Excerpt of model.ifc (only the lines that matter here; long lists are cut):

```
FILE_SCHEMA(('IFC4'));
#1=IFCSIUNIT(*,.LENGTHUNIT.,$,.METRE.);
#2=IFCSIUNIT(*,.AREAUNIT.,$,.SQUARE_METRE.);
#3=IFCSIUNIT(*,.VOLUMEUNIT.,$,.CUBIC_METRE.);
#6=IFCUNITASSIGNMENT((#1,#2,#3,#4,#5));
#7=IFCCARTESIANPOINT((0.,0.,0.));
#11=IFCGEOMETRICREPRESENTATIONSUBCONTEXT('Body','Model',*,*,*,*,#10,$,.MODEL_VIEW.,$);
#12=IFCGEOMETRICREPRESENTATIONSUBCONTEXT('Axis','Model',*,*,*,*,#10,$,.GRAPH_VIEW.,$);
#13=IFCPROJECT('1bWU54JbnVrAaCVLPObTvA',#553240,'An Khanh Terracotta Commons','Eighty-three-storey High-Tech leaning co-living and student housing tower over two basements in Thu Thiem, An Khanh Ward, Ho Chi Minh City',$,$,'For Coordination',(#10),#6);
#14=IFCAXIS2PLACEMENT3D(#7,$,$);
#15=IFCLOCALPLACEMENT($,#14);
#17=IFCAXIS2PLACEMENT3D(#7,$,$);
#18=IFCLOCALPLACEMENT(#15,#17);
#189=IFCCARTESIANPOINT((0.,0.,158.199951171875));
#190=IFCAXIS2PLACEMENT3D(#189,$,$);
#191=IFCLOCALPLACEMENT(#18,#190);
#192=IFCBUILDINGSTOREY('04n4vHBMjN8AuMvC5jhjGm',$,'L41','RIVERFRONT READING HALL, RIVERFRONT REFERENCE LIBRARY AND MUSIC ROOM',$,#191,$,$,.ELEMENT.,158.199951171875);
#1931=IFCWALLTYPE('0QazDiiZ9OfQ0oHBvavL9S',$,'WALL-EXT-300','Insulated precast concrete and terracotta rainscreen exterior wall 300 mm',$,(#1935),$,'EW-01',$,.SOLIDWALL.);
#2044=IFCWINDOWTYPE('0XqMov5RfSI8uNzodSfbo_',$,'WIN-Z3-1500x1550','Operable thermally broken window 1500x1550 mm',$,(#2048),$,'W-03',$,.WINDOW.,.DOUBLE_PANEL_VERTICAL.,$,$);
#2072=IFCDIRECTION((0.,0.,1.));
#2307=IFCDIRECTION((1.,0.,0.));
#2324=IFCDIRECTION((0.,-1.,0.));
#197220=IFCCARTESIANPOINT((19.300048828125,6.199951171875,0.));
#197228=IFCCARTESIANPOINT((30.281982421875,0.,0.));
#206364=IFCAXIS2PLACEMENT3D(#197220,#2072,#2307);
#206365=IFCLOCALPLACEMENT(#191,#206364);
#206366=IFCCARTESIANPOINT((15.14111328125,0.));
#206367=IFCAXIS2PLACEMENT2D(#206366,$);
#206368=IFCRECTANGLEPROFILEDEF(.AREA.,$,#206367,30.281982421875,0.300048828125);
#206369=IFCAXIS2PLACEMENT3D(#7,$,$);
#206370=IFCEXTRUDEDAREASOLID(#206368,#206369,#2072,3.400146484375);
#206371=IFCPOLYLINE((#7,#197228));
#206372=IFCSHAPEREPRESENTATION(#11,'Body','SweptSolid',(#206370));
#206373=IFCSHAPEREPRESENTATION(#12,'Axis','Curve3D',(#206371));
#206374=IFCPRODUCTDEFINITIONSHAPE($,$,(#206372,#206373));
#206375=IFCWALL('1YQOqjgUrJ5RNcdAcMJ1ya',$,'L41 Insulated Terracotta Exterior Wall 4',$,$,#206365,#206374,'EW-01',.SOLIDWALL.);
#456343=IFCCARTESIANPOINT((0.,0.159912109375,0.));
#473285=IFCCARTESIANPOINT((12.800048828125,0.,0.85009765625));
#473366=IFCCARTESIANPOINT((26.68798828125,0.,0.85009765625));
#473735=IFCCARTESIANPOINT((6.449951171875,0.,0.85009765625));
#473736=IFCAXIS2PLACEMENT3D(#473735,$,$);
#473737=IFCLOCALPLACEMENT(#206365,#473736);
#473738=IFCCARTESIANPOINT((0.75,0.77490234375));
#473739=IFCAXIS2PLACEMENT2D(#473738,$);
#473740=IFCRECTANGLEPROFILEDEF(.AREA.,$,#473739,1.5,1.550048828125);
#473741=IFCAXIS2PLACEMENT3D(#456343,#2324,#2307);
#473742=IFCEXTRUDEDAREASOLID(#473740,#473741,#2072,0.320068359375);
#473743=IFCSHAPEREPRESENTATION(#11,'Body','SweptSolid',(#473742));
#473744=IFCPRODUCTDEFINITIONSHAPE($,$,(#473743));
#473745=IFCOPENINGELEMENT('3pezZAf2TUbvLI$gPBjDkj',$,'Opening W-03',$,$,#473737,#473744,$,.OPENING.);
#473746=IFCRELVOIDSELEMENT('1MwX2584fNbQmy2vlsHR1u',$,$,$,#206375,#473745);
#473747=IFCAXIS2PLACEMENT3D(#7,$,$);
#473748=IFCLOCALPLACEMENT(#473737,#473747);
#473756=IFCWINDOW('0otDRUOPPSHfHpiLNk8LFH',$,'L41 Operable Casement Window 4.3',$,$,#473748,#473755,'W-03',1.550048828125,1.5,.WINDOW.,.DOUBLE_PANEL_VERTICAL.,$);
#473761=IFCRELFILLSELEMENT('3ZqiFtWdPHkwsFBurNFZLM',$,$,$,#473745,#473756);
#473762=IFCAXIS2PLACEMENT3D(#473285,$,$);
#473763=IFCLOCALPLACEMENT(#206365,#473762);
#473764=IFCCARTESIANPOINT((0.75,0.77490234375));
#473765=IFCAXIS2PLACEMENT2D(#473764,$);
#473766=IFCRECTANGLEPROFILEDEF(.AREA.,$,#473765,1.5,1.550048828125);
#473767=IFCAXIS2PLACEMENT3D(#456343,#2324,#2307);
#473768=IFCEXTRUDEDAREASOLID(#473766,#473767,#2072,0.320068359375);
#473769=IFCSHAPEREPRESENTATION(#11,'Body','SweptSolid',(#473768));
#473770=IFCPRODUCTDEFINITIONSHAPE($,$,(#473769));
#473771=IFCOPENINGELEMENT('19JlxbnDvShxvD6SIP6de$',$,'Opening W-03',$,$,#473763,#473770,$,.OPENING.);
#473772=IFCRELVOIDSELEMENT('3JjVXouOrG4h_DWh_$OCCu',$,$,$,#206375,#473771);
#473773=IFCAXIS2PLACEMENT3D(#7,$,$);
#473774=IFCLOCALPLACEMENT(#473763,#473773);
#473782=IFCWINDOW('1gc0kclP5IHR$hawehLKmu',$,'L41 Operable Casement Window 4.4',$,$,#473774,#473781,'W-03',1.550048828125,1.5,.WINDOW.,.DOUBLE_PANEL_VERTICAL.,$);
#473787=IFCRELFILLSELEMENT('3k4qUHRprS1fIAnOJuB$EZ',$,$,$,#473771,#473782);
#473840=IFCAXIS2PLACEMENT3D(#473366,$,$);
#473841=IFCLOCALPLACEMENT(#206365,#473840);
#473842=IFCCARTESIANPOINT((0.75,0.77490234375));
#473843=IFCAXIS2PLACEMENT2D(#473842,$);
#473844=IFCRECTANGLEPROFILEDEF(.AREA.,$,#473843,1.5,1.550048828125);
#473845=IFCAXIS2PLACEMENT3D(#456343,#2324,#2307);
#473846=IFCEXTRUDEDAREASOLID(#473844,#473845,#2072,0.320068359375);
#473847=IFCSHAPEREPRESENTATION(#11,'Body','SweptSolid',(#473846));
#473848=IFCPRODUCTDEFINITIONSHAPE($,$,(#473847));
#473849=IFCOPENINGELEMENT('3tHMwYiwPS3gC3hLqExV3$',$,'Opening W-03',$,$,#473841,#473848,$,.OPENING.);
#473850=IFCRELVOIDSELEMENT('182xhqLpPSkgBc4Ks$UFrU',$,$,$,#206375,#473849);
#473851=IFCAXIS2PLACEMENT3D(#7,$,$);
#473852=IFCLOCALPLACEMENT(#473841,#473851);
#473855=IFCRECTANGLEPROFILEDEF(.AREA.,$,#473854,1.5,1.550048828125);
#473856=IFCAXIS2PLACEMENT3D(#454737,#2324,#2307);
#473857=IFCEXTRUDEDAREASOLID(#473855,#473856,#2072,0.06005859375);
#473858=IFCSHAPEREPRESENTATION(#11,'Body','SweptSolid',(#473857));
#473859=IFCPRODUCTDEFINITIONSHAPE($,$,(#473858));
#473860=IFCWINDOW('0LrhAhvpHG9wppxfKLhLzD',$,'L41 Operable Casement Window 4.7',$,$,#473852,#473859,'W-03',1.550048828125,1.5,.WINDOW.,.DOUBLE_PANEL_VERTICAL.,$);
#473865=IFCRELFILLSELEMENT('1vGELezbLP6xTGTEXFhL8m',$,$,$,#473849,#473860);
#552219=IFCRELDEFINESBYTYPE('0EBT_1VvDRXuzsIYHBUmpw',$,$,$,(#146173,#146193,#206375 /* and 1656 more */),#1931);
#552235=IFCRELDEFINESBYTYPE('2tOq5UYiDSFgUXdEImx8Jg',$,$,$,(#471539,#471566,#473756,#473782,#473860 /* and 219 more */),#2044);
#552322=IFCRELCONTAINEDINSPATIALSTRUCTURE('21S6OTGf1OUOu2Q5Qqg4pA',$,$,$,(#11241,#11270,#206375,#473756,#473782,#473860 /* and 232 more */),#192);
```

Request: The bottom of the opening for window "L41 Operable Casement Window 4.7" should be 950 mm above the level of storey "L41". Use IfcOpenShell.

```python
import numpy as np
import ifcopenshell
import ifcopenshell.api.geometry
import ifcopenshell.geom
import ifcopenshell.util.element
import ifcopenshell.util.placement
import ifcopenshell.util.shape
import ifcopenshell.util.unit

model = ifcopenshell.open("model.ifc")
unit_scale = ifcopenshell.util.unit.calculate_unit_scale(model)

window = model.by_guid("0LrhAhvpHG9wppxfKLhLzD")
opening = window.FillsVoids[0].RelatingOpeningElement
storey = ifcopenshell.util.element.get_container(window, ifc_class="IfcBuildingStorey")
level = ifcopenshell.util.placement.get_local_placement(storey.ObjectPlacement)[2, 3]

# The opening's origin need not be at the sill, so measure its lowest point.
shape = ifcopenshell.geom.create_shape(ifcopenshell.geom.settings(), opening)
bottom = ifcopenshell.util.shape.get_shape_bottom_elevation(shape, shape.geometry) / unit_scale
dz = level + 0.95 - bottom

shift = np.array([0.0, 0.0, dz])
# The window is placed relative to its opening, so it follows when the opening moves.
matrix = ifcopenshell.util.placement.get_local_placement(opening.ObjectPlacement)
matrix[:3, 3] += shift
ifcopenshell.api.geometry.edit_object_placement(
    model, product=opening, matrix=matrix, is_si=False, should_transform_children=True
)

print(f"moved by {dz * unit_scale:+.3f} m")

model.write("model_edited.ifc")
```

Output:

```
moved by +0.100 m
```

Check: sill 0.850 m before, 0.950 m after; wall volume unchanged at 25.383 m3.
